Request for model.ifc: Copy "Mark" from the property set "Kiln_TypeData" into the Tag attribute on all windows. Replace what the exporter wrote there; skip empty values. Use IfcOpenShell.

First a look at what the model holds.

```python
import ifcopenshell
import ifcopenshell.util.element

model = ifcopenshell.open("model.ifc")
print(model.schema)
windows = model.by_type("IfcWindow")
print(len(windows), "windows")
for e in windows[:8]:
    source = ifcopenshell.util.element.get_pset(e, "Kiln_TypeData", "Mark")
    target = e.Tag
    print(e.id(), repr(source), repr(target), sep=" | ")
```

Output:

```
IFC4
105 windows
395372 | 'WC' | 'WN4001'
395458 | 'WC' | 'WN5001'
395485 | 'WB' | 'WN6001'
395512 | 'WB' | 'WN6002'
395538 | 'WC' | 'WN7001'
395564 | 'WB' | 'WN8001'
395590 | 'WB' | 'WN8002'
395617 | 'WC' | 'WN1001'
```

```python
import ifcopenshell
import ifcopenshell.util.element

model = ifcopenshell.open("model.ifc")

count = 0
for e in model.by_type("IfcWindow"):
    value = ifcopenshell.util.element.get_pset(e, "Kiln_TypeData", "Mark")
    current = e.Tag
    if not value or not value.strip() or current == value:
        continue
    e.Tag = value
    count += 1

print(count, "windows updated")

model.write("model_rev.ifc")
```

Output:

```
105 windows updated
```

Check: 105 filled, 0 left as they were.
